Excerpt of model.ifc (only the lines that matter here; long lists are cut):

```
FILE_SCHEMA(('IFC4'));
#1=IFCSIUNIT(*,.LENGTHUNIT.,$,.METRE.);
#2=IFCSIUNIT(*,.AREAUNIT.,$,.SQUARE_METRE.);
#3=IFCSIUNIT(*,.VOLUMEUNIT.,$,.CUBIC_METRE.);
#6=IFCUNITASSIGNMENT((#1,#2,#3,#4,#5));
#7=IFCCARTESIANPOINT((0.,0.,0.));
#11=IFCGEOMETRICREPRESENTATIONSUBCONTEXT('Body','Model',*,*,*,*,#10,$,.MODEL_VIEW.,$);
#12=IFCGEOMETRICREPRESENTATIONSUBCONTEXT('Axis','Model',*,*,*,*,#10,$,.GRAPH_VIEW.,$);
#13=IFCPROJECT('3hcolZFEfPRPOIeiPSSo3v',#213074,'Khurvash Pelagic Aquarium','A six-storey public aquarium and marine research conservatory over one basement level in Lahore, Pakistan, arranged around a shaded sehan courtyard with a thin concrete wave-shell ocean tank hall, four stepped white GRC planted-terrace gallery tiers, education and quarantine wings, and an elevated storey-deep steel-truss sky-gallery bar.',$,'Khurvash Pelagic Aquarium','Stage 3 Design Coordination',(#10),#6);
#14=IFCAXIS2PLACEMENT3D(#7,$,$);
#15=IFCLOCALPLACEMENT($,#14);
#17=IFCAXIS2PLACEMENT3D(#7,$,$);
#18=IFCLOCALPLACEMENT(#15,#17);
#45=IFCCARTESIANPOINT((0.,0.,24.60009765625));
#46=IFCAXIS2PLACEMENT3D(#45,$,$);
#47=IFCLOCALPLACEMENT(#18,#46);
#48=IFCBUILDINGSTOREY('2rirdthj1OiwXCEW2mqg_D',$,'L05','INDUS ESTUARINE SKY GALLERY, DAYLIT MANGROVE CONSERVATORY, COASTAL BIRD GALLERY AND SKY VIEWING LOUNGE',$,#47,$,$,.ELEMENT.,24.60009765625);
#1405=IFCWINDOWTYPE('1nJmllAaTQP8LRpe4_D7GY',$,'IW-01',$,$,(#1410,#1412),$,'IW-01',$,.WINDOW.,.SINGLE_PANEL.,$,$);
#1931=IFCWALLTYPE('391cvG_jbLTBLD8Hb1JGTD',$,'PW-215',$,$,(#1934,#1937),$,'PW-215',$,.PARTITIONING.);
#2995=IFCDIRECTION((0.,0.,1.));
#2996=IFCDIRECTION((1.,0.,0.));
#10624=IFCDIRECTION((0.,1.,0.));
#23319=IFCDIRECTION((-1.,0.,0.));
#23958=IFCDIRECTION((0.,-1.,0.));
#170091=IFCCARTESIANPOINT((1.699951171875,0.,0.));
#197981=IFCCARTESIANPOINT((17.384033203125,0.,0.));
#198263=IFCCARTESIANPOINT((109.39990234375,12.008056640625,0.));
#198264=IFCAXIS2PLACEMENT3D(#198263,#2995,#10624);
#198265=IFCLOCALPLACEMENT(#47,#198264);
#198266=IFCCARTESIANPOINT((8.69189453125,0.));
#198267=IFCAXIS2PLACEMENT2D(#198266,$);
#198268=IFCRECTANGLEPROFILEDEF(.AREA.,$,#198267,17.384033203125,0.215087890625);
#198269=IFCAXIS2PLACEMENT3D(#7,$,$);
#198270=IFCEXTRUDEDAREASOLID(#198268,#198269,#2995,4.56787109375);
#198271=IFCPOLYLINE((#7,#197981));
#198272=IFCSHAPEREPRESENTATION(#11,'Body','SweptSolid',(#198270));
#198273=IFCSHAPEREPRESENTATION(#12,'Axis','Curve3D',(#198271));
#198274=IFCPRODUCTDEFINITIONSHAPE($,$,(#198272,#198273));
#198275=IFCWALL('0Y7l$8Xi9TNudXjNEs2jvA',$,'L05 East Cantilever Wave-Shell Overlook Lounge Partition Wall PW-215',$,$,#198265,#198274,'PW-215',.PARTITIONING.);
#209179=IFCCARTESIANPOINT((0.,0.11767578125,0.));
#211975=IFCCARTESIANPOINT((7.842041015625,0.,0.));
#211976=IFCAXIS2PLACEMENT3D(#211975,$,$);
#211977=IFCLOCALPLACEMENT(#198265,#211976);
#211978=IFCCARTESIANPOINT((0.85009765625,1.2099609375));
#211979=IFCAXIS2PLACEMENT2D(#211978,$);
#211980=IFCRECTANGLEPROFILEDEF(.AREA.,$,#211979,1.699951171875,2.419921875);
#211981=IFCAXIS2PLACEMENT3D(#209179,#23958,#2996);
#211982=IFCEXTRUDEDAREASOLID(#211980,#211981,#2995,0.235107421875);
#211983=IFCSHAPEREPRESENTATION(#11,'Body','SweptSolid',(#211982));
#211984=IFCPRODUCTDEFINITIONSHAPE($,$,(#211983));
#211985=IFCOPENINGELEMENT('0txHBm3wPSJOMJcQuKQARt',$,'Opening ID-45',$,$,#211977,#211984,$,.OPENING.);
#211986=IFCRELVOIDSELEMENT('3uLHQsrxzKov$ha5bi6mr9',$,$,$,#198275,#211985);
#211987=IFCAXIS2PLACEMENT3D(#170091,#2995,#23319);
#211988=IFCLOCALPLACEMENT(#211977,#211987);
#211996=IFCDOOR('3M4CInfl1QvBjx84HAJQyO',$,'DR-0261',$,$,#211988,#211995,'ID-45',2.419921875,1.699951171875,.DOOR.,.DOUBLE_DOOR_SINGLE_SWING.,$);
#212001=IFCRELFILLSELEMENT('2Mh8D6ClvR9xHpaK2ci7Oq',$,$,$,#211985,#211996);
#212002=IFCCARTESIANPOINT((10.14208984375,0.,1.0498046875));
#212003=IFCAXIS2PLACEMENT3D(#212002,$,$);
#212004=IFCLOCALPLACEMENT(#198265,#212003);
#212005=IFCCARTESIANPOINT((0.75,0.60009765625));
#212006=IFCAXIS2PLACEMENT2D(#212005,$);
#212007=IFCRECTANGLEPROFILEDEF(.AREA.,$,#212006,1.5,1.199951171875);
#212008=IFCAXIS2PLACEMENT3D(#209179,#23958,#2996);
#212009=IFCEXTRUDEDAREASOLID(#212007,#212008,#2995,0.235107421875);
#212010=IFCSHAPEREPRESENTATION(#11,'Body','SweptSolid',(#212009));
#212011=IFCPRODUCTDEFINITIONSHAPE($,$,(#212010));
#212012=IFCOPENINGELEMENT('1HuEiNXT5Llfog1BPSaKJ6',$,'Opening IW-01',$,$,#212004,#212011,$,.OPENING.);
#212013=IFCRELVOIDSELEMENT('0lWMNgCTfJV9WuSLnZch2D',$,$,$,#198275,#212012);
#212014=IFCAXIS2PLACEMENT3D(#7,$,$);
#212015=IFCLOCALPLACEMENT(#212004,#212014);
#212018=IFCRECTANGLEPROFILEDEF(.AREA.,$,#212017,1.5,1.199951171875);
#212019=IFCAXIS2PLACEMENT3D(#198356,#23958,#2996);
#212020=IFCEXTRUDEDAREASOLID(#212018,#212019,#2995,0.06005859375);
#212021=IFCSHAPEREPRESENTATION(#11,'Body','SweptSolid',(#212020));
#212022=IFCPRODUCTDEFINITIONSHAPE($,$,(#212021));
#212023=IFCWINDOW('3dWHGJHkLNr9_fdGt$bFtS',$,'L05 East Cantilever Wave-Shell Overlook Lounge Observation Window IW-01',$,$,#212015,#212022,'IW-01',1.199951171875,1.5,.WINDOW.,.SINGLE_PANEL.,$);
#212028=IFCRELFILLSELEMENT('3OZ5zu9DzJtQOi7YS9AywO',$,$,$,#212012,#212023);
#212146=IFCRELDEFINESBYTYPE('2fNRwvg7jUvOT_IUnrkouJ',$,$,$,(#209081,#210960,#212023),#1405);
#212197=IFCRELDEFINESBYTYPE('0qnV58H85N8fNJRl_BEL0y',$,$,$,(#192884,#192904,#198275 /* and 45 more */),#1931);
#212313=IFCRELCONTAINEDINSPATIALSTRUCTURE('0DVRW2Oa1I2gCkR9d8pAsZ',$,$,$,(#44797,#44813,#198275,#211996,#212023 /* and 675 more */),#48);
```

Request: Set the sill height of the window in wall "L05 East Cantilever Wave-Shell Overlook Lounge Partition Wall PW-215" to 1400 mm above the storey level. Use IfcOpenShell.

```python
import numpy as np
import ifcopenshell
import ifcopenshell.api.geometry
import ifcopenshell.geom
import ifcopenshell.util.element
import ifcopenshell.util.placement
import ifcopenshell.util.shape
import ifcopenshell.util.unit

model = ifcopenshell.open("model.ifc")
unit_scale = ifcopenshell.util.unit.calculate_unit_scale(model)

window = model.by_guid("3dWHGJHkLNr9_fdGt$bFtS")
opening = window.FillsVoids[0].RelatingOpeningElement
storey = ifcopenshell.util.element.get_container(window, ifc_class="IfcBuildingStorey")
level = ifcopenshell.util.placement.get_local_placement(storey.ObjectPlacement)[2, 3]

# The opening's origin need not be at the sill, so measure its lowest point.
shape = ifcopenshell.geom.create_shape(ifcopenshell.geom.settings(), opening)
bottom = ifcopenshell.util.shape.get_shape_bottom_elevation(shape, shape.geometry) / unit_scale
dz = level + 1.4 - bottom

shift = np.array([0.0, 0.0, dz])
# The window is placed relative to its opening, so it follows when the opening moves.
matrix = ifcopenshell.util.placement.get_local_placement(opening.ObjectPlacement)
matrix[:3, 3] += shift
ifcopenshell.api.geometry.edit_object_placement(
    model, product=opening, matrix=matrix, is_si=False, should_transform_children=True
)

print(f"moved by {dz * unit_scale:+.3f} m")

model.write("model_rev.ifc")
```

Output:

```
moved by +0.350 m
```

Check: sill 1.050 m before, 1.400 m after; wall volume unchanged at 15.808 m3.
